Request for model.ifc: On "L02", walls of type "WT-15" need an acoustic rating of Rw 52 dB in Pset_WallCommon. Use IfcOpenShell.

First a look at what the model holds.

```python
import ifcopenshell
import ifcopenshell.util.element

model = ifcopenshell.open("model.ifc")
print(model.schema)
storey = next(s for s in model.by_type("IfcBuildingStorey") if s.Name == "L02")
walls = [e for e in ifcopenshell.util.element.get_decomposition(storey) if e.is_a("IfcWall")]
seen = {}
for e in walls:
    element_type = ifcopenshell.util.element.get_type(e)
    key = (element_type.Name if element_type != e and element_type else None, ifcopenshell.util.element.get_pset(e, "Pset_WallCommon", "AcousticRating"))
    seen[key] = seen.get(key, 0) + 1
for (name, value), count in sorted(seen.items(), key=str):
    print(count, "x", name, "|", value)
```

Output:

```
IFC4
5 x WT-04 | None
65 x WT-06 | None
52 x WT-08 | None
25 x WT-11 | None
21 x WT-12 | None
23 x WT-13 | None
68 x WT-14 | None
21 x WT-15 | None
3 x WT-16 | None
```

```python
import ifcopenshell
import ifcopenshell.api.pset
import ifcopenshell.util.element

model = ifcopenshell.open("model.ifc")

storey = next(s for s in model.by_type("IfcBuildingStorey") if s.Name == "L02")
walls = [e for e in ifcopenshell.util.element.get_decomposition(storey) if e.is_a("IfcWall")]

count = 0
for e in walls:
    element_type = ifcopenshell.util.element.get_type(e)
    if element_type in (None, e) or element_type.Name != "WT-15":
        continue
    # add_pset returns the element's existing set when there is one.
    pset = ifcopenshell.api.pset.add_pset(model, product=e, name="Pset_WallCommon")
    ifcopenshell.api.pset.edit_pset(model, pset=pset, properties={"AcousticRating": "Rw 52 dB"})
    count += 1

print(count, "walls updated")

model.write("model_rev.ifc")
```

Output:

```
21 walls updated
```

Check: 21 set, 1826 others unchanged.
